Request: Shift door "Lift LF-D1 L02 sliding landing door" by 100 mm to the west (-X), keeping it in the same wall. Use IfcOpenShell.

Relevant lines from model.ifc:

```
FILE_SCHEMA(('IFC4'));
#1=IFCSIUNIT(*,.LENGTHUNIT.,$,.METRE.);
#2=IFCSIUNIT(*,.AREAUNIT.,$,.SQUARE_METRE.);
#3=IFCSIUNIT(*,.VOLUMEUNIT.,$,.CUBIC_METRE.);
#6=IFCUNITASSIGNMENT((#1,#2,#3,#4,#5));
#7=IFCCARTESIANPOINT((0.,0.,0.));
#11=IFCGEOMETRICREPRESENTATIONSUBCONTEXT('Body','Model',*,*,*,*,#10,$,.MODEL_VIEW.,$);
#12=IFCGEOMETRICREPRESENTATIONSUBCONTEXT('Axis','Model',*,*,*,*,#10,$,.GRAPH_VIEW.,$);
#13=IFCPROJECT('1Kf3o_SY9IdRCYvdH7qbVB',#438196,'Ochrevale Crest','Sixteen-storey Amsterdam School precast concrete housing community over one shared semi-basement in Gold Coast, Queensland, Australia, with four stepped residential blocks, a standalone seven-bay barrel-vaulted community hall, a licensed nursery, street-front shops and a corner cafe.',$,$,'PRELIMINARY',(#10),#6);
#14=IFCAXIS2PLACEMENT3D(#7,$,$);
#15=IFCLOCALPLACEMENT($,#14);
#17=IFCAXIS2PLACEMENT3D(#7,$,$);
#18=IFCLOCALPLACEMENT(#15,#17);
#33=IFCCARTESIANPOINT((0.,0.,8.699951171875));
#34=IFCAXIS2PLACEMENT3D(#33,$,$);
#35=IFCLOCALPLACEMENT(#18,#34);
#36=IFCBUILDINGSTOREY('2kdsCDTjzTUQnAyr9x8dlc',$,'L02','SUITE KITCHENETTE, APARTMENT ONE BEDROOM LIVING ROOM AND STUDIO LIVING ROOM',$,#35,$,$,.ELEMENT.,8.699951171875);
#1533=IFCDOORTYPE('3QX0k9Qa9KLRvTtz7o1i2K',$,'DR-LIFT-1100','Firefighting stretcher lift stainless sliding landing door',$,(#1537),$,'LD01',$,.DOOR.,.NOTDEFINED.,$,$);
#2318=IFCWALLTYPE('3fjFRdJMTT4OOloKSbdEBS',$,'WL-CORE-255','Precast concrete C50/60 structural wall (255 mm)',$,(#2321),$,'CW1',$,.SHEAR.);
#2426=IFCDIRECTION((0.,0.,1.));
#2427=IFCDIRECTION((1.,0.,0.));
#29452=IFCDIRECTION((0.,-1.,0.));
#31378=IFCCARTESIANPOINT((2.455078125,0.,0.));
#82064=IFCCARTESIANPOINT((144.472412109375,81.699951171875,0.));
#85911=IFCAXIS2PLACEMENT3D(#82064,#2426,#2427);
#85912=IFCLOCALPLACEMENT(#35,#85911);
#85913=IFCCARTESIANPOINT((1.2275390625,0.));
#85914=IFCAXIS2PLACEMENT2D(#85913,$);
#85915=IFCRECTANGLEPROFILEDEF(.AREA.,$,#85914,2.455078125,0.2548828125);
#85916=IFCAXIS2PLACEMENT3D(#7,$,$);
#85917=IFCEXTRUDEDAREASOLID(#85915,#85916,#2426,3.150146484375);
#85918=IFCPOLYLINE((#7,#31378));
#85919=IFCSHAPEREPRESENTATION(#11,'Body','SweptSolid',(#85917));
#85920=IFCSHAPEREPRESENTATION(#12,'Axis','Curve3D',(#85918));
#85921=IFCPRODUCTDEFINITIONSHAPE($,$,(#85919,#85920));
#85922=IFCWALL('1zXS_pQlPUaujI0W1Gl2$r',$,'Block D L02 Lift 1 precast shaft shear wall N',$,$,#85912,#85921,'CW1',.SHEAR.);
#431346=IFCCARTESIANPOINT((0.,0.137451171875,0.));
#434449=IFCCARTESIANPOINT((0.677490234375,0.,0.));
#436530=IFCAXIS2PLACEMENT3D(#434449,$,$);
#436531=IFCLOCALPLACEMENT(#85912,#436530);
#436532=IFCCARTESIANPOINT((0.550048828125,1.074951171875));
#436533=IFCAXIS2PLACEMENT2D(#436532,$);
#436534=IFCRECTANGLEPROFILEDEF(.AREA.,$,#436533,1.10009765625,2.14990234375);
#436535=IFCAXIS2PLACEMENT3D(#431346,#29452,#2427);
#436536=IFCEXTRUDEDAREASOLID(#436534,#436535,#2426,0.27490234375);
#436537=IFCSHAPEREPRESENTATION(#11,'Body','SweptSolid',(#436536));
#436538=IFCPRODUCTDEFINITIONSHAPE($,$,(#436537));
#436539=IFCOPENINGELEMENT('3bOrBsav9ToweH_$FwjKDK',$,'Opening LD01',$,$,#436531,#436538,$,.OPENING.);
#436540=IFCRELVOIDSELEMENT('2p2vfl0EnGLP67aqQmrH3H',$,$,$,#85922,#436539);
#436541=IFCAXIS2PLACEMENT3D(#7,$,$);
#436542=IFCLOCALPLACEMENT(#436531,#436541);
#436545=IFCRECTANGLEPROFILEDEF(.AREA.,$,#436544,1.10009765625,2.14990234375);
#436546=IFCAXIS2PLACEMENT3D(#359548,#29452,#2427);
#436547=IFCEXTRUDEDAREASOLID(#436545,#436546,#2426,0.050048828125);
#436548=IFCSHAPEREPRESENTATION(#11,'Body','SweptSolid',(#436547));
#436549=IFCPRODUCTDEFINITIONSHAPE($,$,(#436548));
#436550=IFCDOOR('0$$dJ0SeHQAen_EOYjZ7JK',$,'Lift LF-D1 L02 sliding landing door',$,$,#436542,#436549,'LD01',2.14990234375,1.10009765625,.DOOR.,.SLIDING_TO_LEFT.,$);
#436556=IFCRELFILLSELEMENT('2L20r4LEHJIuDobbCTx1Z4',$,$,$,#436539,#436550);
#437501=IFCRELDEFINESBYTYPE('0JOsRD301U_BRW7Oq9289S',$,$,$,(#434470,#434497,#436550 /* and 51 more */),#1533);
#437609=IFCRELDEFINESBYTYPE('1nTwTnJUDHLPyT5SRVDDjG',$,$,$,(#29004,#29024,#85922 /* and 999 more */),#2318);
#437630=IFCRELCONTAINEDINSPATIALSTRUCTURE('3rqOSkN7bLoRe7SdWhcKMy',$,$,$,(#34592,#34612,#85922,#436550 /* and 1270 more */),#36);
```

```python
import ifcopenshell
import ifcopenshell.api.geometry
import ifcopenshell.util.placement
import ifcopenshell.util.unit

model = ifcopenshell.open("model.ifc")
unit_scale = ifcopenshell.util.unit.calculate_unit_scale(model)

door = model.by_id(436550)
opening = door.FillsVoids[0].RelatingOpeningElement
wall = opening.VoidsElements[0].RelatingBuildingElement

wall_matrix = ifcopenshell.util.placement.get_local_placement(wall.ObjectPlacement)
shift = wall_matrix[:3, 0] * -0.1 / unit_scale
before = ifcopenshell.util.placement.get_local_placement(door.ObjectPlacement)[:3, 3].copy()

# The door is placed relative to its opening, so it follows when the opening moves.
matrix = ifcopenshell.util.placement.get_local_placement(opening.ObjectPlacement)
matrix[:3, 3] += shift
ifcopenshell.api.geometry.edit_object_placement(
    model, product=opening, matrix=matrix, is_si=False, should_transform_children=True
)

after = ifcopenshell.util.placement.get_local_placement(door.ObjectPlacement)[:3, 3]
print("door moved by", (after - before).round(3) + 0.0)

model.write("model_updated.ifc")
```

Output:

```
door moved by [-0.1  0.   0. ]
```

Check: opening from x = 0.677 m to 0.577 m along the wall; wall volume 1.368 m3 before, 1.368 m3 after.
